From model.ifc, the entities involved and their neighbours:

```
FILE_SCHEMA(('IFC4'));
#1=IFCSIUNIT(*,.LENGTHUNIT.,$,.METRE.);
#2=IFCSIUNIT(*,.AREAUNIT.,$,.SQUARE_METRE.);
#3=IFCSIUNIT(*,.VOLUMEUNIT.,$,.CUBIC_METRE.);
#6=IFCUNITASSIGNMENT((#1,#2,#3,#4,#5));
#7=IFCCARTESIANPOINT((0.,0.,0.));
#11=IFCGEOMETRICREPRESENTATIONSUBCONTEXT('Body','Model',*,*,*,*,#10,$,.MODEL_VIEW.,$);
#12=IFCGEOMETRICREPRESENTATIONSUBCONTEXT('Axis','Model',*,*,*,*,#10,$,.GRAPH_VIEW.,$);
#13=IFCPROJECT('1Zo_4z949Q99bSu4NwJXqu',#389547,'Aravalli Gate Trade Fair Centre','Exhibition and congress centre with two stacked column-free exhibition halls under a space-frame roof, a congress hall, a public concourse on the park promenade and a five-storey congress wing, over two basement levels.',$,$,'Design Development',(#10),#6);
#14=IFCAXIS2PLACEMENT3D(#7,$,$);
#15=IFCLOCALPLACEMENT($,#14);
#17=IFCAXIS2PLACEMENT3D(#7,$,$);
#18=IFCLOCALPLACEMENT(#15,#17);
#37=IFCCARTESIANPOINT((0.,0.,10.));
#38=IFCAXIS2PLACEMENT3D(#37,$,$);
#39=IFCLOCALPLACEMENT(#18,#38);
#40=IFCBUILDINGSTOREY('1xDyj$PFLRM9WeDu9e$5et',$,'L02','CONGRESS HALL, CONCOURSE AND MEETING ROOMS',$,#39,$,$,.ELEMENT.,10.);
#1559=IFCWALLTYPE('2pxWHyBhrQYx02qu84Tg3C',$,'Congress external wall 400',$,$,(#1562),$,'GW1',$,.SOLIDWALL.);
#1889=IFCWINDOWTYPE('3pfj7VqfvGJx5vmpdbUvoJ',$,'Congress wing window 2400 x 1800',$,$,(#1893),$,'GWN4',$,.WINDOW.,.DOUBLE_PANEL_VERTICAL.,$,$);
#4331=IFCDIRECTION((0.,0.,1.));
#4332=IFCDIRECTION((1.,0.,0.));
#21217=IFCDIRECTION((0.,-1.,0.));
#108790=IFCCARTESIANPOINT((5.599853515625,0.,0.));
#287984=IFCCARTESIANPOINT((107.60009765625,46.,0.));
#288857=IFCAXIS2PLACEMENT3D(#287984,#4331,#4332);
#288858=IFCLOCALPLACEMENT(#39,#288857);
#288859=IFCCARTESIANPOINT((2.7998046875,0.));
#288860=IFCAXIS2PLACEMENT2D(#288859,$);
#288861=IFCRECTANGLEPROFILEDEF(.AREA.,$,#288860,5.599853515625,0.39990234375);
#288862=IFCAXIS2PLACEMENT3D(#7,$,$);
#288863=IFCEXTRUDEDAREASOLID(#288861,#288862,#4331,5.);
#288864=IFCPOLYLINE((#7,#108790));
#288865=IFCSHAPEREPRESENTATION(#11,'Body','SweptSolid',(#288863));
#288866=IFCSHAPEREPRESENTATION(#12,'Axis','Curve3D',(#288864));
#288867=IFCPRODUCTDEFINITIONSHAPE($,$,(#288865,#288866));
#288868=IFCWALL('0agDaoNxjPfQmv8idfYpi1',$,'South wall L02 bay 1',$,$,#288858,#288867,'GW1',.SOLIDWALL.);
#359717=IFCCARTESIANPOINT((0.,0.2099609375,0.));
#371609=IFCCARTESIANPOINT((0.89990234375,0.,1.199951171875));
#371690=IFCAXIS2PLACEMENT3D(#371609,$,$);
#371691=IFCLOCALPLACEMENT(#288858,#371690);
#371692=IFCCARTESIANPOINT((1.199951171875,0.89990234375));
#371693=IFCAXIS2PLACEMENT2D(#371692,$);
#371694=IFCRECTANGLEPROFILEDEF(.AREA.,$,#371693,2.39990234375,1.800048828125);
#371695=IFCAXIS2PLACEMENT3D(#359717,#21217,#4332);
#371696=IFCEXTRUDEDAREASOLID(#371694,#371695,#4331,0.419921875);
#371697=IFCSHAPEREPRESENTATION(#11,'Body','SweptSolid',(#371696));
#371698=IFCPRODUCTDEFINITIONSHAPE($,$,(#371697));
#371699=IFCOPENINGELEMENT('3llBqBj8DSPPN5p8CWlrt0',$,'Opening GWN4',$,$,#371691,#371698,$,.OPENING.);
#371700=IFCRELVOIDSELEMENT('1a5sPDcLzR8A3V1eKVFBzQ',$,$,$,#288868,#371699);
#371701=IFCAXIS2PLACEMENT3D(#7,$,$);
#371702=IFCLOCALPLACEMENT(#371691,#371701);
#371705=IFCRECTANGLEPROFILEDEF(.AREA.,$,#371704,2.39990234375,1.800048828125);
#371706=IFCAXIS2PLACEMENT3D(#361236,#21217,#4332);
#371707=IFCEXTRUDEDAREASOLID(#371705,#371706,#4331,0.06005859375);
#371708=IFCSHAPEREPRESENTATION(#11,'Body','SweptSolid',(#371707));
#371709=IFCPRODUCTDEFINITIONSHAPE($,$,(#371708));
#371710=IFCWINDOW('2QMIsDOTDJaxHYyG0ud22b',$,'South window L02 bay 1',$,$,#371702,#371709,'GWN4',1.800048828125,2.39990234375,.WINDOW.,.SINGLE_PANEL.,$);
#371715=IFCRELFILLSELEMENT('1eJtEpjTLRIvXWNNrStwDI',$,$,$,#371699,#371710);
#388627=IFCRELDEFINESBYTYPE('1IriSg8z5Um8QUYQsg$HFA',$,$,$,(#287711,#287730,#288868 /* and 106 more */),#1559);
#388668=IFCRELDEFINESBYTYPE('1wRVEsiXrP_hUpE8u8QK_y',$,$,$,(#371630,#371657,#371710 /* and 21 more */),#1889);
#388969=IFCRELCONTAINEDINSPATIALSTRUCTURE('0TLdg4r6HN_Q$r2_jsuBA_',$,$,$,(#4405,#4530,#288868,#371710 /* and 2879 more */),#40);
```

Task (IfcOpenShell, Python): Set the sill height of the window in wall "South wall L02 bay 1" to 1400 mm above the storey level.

```python
import numpy as np
import ifcopenshell
import ifcopenshell.api.geometry
import ifcopenshell.geom
import ifcopenshell.util.element
import ifcopenshell.util.placement
import ifcopenshell.util.shape
import ifcopenshell.util.unit

model = ifcopenshell.open("model.ifc")
unit_scale = ifcopenshell.util.unit.calculate_unit_scale(model)

window = model.by_guid("2QMIsDOTDJaxHYyG0ud22b")
opening = window.FillsVoids[0].RelatingOpeningElement
storey = ifcopenshell.util.element.get_container(window, ifc_class="IfcBuildingStorey")
level = ifcopenshell.util.placement.get_local_placement(storey.ObjectPlacement)[2, 3]

# The opening's origin need not be at the sill, so measure its lowest point.
shape = ifcopenshell.geom.create_shape(ifcopenshell.geom.settings(), opening)
bottom = ifcopenshell.util.shape.get_shape_bottom_elevation(shape, shape.geometry) / unit_scale
dz = level + 1.4 / unit_scale - bottom

shift = np.array([0.0, 0.0, dz])
# The window is placed relative to its opening, so it follows when the opening moves.
matrix = ifcopenshell.util.placement.get_local_placement(opening.ObjectPlacement)
matrix[:3, 3] += shift
ifcopenshell.api.geometry.edit_object_placement(
    model, product=opening, matrix=matrix, is_si=False, should_transform_children=True
)

print(f"moved by {dz * unit_scale:+.3f} m")

model.write("model_updated.ifc")
```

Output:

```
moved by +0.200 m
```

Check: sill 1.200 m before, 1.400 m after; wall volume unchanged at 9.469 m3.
